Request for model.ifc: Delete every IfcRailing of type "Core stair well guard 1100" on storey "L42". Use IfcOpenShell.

First a look at what the model holds.

```python
import ifcopenshell
import ifcopenshell.util.element

model = ifcopenshell.open("model.ifc")
print(model.schema)
storey = next(s for s in model.by_type("IfcBuildingStorey") if s.Name == "L42")
railings = [e for e in ifcopenshell.util.element.get_decomposition(storey) if e.is_a("IfcRailing")]
seen = {}
for e in railings:
    element_type = ifcopenshell.util.element.get_type(e)
    name = element_type.Name if element_type not in (None, e) else None
    seen[name] = seen.get(name, 0) + 1
for name, count in sorted(seen.items(), key=str):
    print(count, "x", name)
```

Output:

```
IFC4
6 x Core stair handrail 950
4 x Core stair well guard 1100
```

```python
import ifcopenshell
import ifcopenshell.api.root
import ifcopenshell.util.element

model = ifcopenshell.open("model.ifc")

storey = next(s for s in model.by_type("IfcBuildingStorey") if s.Name == "L42")
railings = [e for e in ifcopenshell.util.element.get_decomposition(storey) if e.is_a("IfcRailing")]
targets = [e for e in railings if (t := ifcopenshell.util.element.get_type(e)) not in (None, e) and t.Name == "Core stair well guard 1100"]

for e in targets:
    ifcopenshell.api.root.remove_product(model, product=e)
print(len(targets), "removed")

model.write("model_edited.ifc")
```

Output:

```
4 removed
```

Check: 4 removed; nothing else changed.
